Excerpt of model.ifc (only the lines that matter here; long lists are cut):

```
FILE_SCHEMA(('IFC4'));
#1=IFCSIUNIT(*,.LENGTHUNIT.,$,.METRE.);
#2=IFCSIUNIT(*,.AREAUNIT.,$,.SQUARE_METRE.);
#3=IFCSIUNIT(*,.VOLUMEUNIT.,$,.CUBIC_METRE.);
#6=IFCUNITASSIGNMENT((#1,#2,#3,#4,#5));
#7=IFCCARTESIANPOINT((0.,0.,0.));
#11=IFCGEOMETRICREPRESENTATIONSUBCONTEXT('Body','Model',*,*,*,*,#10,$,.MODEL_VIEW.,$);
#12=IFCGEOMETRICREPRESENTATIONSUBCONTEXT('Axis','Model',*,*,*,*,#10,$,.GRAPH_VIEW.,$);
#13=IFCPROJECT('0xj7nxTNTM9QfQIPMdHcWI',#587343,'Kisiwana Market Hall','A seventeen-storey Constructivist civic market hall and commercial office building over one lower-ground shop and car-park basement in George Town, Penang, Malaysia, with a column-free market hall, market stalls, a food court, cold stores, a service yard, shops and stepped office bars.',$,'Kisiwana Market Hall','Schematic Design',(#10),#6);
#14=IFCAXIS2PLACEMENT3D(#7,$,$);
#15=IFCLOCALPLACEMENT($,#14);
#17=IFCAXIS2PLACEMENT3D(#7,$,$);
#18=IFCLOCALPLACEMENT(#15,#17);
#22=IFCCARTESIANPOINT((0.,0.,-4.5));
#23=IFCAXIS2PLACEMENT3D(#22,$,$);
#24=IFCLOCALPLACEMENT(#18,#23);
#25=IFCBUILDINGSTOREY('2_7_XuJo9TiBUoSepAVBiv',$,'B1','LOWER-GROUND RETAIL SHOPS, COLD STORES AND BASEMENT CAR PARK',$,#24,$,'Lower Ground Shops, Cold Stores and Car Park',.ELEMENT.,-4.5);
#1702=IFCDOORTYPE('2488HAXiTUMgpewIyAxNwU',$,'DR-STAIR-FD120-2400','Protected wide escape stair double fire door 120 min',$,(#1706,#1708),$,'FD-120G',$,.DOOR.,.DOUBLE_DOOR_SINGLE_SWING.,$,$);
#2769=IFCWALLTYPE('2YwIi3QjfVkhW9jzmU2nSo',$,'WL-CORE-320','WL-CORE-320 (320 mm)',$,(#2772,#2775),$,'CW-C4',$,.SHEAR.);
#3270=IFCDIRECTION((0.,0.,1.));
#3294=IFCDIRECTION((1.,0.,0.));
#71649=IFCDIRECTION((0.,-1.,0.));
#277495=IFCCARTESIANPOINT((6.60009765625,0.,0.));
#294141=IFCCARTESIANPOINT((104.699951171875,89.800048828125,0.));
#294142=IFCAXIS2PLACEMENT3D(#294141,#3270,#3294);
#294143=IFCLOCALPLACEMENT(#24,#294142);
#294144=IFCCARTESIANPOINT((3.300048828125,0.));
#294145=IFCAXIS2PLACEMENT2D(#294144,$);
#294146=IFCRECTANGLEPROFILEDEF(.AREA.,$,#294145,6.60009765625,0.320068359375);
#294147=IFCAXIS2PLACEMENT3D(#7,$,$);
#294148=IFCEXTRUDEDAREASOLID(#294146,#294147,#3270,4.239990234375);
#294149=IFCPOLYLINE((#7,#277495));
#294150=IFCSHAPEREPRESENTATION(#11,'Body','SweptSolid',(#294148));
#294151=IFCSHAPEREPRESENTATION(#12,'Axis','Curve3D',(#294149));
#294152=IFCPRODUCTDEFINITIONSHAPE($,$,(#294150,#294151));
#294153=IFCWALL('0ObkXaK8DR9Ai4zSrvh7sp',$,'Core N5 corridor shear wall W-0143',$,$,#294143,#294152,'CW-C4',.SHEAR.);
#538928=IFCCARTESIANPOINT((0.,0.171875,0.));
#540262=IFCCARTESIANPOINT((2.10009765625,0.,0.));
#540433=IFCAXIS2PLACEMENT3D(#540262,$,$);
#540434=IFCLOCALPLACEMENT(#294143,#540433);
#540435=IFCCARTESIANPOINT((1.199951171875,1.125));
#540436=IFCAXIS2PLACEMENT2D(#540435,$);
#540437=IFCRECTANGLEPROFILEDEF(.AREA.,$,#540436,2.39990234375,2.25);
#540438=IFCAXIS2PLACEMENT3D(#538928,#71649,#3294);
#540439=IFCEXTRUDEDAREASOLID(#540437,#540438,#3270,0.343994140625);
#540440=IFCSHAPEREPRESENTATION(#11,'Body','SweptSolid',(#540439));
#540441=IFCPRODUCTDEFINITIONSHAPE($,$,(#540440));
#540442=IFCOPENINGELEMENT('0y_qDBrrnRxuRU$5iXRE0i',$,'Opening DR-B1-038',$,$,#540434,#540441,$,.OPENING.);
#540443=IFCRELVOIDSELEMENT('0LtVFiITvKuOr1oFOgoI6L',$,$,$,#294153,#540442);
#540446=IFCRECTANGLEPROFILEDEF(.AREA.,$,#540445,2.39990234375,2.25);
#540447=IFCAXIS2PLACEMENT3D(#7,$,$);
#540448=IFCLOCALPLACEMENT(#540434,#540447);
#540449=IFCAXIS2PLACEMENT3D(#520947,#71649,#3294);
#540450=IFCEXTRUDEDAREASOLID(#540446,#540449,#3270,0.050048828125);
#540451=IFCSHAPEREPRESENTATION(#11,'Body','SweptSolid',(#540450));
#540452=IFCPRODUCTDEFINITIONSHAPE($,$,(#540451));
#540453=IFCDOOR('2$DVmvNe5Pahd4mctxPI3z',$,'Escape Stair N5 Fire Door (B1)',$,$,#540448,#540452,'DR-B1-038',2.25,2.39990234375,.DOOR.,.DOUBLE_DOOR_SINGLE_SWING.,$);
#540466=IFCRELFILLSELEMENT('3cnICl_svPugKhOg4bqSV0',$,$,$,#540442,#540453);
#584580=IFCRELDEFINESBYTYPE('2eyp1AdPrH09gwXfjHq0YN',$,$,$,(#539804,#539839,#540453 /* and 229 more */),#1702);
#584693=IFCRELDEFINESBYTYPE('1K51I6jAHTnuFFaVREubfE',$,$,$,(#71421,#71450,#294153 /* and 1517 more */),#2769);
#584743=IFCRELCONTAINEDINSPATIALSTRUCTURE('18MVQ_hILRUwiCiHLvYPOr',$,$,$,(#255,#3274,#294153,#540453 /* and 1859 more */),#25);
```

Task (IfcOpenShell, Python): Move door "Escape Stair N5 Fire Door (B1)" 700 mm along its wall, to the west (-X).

```python
import ifcopenshell
import ifcopenshell.api.geometry
import ifcopenshell.util.placement
import ifcopenshell.util.unit

model = ifcopenshell.open("model.ifc")
unit_scale = ifcopenshell.util.unit.calculate_unit_scale(model)

door = model.by_guid("2$DVmvNe5Pahd4mctxPI3z")
opening = door.FillsVoids[0].RelatingOpeningElement
wall = opening.VoidsElements[0].RelatingBuildingElement

wall_matrix = ifcopenshell.util.placement.get_local_placement(wall.ObjectPlacement)
shift = wall_matrix[:3, 0] * -0.7 / unit_scale
before = ifcopenshell.util.placement.get_local_placement(door.ObjectPlacement)[:3, 3].copy()

# The door is placed relative to its opening, so it follows when the opening moves.
matrix = ifcopenshell.util.placement.get_local_placement(opening.ObjectPlacement)
matrix[:3, 3] += shift
ifcopenshell.api.geometry.edit_object_placement(
    model, product=opening, matrix=matrix, is_si=False, should_transform_children=True
)

after = ifcopenshell.util.placement.get_local_placement(door.ObjectPlacement)[:3, 3]
print("door moved by", (after - before).round(3) + 0.0)

model.write("model_rev.ifc")
```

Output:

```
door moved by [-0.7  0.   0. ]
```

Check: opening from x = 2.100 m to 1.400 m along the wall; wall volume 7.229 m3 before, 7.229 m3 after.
